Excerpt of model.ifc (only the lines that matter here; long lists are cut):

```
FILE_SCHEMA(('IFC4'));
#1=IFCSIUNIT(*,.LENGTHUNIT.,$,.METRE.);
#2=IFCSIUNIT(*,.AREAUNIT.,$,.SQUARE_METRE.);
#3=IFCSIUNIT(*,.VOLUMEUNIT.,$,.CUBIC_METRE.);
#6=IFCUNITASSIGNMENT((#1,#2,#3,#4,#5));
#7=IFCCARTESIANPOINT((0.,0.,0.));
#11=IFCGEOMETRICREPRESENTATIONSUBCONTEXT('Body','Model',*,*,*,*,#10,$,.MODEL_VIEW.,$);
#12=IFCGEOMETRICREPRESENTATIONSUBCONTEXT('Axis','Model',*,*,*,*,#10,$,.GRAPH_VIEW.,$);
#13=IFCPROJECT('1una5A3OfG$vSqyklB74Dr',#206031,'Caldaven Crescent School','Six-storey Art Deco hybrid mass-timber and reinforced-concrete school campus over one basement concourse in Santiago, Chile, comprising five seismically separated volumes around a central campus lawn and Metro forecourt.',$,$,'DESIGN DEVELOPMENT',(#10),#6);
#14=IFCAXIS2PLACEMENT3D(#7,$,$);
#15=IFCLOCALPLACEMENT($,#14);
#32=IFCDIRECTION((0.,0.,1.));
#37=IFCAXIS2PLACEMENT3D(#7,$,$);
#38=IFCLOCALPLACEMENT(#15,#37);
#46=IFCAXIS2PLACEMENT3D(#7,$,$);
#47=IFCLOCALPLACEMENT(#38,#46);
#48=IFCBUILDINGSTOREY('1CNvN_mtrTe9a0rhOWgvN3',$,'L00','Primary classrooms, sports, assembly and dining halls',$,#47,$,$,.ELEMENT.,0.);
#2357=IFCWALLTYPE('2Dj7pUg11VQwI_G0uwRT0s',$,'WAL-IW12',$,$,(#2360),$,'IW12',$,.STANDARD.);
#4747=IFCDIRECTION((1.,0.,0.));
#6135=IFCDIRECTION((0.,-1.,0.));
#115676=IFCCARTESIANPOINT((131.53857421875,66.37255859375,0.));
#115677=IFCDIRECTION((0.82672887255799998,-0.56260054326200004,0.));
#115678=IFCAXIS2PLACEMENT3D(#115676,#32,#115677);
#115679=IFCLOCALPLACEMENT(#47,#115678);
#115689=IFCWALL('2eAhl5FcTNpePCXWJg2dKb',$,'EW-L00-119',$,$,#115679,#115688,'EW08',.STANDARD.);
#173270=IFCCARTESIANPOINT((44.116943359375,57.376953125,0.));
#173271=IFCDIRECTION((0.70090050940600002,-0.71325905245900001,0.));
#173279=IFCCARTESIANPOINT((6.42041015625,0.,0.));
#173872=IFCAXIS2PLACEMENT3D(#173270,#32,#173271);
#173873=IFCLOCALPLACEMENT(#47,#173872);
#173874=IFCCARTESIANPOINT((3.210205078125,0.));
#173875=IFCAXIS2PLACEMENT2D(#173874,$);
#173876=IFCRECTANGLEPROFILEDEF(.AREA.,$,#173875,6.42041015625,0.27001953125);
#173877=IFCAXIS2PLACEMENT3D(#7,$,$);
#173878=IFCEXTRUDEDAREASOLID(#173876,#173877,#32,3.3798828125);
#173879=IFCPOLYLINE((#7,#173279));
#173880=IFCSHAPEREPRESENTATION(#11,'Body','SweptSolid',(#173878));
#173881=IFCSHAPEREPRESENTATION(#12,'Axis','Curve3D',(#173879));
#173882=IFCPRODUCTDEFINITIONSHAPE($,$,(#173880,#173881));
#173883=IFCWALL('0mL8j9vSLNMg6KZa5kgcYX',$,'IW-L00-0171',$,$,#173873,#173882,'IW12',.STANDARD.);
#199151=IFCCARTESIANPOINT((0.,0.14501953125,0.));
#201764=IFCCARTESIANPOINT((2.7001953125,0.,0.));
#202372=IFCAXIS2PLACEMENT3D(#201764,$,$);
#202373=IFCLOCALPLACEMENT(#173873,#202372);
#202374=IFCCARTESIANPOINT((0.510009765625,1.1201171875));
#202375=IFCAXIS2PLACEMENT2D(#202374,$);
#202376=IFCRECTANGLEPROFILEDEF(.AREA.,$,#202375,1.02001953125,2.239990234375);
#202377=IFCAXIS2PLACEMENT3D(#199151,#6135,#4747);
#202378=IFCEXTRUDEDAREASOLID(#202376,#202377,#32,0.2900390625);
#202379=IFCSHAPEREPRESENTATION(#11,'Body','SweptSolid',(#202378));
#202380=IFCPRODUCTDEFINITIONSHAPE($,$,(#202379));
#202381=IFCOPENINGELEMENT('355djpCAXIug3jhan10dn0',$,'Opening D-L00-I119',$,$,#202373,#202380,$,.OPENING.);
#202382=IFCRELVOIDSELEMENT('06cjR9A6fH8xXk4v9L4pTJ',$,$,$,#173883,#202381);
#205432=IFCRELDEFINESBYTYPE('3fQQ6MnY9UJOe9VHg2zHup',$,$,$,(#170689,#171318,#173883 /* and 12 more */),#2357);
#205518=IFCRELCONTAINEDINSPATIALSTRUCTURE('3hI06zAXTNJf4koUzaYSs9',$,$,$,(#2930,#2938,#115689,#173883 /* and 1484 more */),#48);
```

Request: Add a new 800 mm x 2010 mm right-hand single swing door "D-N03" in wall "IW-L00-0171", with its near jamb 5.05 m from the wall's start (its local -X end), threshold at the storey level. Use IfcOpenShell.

```python
import numpy as np
import ifcopenshell
import ifcopenshell.api.feature
import ifcopenshell.api.geometry
import ifcopenshell.api.root
import ifcopenshell.api.spatial
import ifcopenshell.geom
import ifcopenshell.util.element
import ifcopenshell.util.placement
import ifcopenshell.util.representation
import ifcopenshell.util.shape
import ifcopenshell.util.unit

model = ifcopenshell.open("model.ifc")
unit_scale = ifcopenshell.util.unit.calculate_unit_scale(model)
settings = ifcopenshell.geom.settings()


def volume(element):
    """Net volume in cubic metres, openings subtracted."""
    shape = ifcopenshell.geom.create_shape(settings, element)
    return ifcopenshell.util.shape.get_volume(shape.geometry)


wall = model.by_id(173883)
storey = ifcopenshell.util.element.get_container(wall, ifc_class="IfcBuildingStorey")
context = ifcopenshell.util.representation.get_context(model, "Model", "Body", "MODEL_VIEW")
before = volume(wall)

width, height, from_end, sill = 0.8, 2.01, 5.05, 0.0  # metres

# The wall runs along its own X axis, and the end named is its -X end.
wall_shape = ifcopenshell.geom.create_shape(settings, wall)
x, y, z = ifcopenshell.util.shape.get_vertices(wall_shape.geometry).T
start = x.min() + from_end
face, thickness = float(y.min()), float(y.max() - y.min())
wall_matrix = ifcopenshell.util.placement.get_local_placement(wall.ObjectPlacement)
level = ifcopenshell.util.placement.get_local_placement(storey.ObjectPlacement)[2, 3]


def in_wall(x, y):
    """Placement at x, y metres in the wall's axes, at sill height."""
    matrix = wall_matrix.copy()
    matrix[:, 3] = wall_matrix @ np.array([x / unit_scale, y / unit_scale, 0.0, 1.0])
    matrix[2, 3] = level + sill / unit_scale
    return matrix


# Opening: a box that overshoots both wall faces by 50 mm.
opening = ifcopenshell.api.root.create_entity(model, ifc_class="IfcOpeningElement", predefined_type="OPENING")
box = ifcopenshell.api.geometry.add_wall_representation(
    model, context=context, length=width, height=height, thickness=thickness + 0.1
)
ifcopenshell.api.geometry.assign_representation(model, product=opening, representation=box)
ifcopenshell.api.geometry.edit_object_placement(model, product=opening, matrix=in_wall(start, face - 0.05), is_si=False)
ifcopenshell.api.feature.add_feature(model, feature=opening, element=wall)

door = ifcopenshell.api.root.create_entity(model, ifc_class="IfcDoor", name="D-N03", predefined_type="DOOR")
door.OverallWidth, door.OverallHeight = width / unit_scale, height / unit_scale
door.OperationType = "SINGLE_SWING_RIGHT"
body = ifcopenshell.api.geometry.add_door_representation(
    model,
    context=context,
    overall_width=door.OverallWidth,
    overall_height=door.OverallHeight,
    operation_type="SINGLE_SWING_RIGHT",
    lining_properties={"LiningDepth": thickness / unit_scale, "ThresholdDepth": thickness / unit_scale},
)
ifcopenshell.api.geometry.assign_representation(model, product=door, representation=body)
ifcopenshell.api.spatial.assign_container(model, products=[door], relating_structure=storey)
ifcopenshell.api.feature.add_filling(model, opening=opening, element=door)

# The lining spans the wall, so the door starts at the wall face.
ifcopenshell.api.geometry.edit_object_placement(model, product=door, matrix=in_wall(start, face), is_si=False)

after = volume(wall)

print(f"wall volume {before:.3f} -> {after:.3f} m3")

model.write("model_rev.ifc")
```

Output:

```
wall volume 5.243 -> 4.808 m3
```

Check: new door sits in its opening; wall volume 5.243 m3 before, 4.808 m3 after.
